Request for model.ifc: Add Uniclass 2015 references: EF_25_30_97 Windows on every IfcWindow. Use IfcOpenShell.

First a look at what the model holds.

```python
import ifcopenshell

model = ifcopenshell.open("model.ifc")
print(model.schema)
print("classifications:", [c.Name for c in model.by_type("IfcClassification")])
for ifc_class in ("IfcDoor", "IfcRoof", "IfcStair", "IfcWall", "IfcWindow"):
    print(ifc_class, len(model.by_type(ifc_class)))
```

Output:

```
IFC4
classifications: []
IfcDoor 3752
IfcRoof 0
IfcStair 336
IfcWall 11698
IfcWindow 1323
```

```python
import ifcopenshell
import ifcopenshell.api.classification

model = ifcopenshell.open("model.ifc")

system = ifcopenshell.api.classification.add_classification(model, classification="Uniclass 2015")

codes = {
    "IfcWindow": ("EF_25_30_97", "Windows"),
}
for ifc_class, (code, name) in codes.items():
    products = model.by_type(ifc_class)
    ifcopenshell.api.classification.add_reference(
        model, products=products, classification=system, identification=code, name=name
    )
    print(code, len(products))

model.write("model_v2.ifc")
```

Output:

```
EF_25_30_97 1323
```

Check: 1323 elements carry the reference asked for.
